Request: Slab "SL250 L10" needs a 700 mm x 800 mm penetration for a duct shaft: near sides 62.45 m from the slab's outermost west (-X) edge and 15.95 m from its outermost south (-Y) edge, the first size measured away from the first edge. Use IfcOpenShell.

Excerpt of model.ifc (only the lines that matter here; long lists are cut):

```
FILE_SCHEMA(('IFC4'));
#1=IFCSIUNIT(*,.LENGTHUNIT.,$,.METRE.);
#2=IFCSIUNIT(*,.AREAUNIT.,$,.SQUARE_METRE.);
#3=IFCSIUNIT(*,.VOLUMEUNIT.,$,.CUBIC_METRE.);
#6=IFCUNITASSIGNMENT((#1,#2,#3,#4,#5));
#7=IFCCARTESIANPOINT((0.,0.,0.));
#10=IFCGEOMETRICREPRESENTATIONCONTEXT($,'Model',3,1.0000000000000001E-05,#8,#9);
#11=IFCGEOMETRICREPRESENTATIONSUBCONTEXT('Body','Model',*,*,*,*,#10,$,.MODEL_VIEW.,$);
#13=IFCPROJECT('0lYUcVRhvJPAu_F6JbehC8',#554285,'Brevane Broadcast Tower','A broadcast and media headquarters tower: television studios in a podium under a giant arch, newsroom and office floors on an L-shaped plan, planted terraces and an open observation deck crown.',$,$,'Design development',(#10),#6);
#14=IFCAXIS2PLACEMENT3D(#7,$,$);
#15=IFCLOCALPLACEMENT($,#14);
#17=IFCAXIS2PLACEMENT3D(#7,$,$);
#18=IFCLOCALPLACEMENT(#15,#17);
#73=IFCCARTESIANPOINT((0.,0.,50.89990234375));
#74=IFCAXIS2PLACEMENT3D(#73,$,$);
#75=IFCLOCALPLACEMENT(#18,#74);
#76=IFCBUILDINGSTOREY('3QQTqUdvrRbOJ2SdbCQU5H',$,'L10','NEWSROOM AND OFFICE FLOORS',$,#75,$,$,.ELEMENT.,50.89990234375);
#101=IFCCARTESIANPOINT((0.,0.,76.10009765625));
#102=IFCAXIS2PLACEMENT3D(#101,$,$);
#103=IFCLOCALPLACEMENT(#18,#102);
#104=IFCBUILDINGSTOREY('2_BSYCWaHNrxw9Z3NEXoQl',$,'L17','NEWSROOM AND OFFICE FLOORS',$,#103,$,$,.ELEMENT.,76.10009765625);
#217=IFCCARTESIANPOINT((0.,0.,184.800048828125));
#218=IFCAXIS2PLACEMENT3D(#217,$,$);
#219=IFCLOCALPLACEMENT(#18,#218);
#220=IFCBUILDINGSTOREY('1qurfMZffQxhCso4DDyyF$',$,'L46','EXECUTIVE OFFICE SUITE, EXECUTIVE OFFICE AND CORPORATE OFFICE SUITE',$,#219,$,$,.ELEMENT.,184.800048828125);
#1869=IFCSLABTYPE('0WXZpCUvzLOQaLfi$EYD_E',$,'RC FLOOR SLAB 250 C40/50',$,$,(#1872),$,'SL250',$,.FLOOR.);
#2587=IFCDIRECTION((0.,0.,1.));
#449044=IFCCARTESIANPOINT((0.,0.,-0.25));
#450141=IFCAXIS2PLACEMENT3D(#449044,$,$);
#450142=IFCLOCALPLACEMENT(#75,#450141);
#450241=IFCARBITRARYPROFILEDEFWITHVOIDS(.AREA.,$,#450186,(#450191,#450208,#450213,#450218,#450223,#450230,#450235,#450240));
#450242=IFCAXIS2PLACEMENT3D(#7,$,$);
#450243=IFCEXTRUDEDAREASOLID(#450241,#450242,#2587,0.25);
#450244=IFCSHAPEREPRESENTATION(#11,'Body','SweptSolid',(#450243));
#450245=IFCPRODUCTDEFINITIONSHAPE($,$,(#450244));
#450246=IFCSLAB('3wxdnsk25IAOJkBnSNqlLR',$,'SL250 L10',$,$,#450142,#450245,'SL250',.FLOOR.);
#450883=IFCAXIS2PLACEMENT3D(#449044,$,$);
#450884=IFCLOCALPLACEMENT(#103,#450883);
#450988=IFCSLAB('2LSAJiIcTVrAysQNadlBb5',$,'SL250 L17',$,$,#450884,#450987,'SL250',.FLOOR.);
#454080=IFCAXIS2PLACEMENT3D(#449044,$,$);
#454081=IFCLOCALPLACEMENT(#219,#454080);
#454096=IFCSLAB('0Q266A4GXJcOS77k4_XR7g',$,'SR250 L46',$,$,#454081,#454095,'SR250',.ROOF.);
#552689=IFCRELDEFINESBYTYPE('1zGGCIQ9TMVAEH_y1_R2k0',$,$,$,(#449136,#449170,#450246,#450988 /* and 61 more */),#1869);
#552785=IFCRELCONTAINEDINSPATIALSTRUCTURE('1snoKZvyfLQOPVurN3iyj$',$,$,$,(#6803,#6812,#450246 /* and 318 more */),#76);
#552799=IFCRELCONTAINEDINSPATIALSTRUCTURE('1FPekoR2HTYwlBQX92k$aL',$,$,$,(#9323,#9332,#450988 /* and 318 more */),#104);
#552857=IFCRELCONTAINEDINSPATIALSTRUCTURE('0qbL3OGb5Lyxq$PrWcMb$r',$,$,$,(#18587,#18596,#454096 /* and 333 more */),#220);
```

```python
import numpy as np
import ifcopenshell
import ifcopenshell.api.feature
import ifcopenshell.api.geometry
import ifcopenshell.api.root
import ifcopenshell.geom
import ifcopenshell.util.placement
import ifcopenshell.util.representation
import ifcopenshell.util.shape
import ifcopenshell.util.unit

model = ifcopenshell.open("model.ifc")
unit_scale = ifcopenshell.util.unit.calculate_unit_scale(model)
settings = ifcopenshell.geom.settings()


def volume(element):
    """Net volume in cubic metres, openings subtracted."""
    shape = ifcopenshell.geom.create_shape(settings, element)
    return ifcopenshell.util.shape.get_volume(shape.geometry)


slab = model.by_id(450246)
before = volume(slab)

# Extent in the slab's own axes, in metres. The edges named are its -X and -Y sides.
slab_shape = ifcopenshell.geom.create_shape(settings, slab)
vertices = ifcopenshell.util.shape.get_vertices(slab_shape.geometry)
x_min, y_min, bottom = vertices.min(axis=0)
top = vertices[:, 2].max()

opening = ifcopenshell.api.root.create_entity(model, ifc_class="IfcOpeningElement", name="Duct shaft opening", predefined_type="OPENING")
context = ifcopenshell.util.representation.get_context(model, "Model", "Body", "MODEL_VIEW")
width, depth = 0.7, 0.8
outline = [(0.0, 0.0), (width, 0.0), (width, depth), (0.0, depth), (0.0, 0.0)]
# Overshoot both faces by 50 mm so the cut is clean.
shape = ifcopenshell.api.geometry.add_slab_representation(
    model, context=context, depth=top - bottom + 0.1, polyline=outline
)
ifcopenshell.api.geometry.assign_representation(model, product=opening, representation=shape)

matrix = ifcopenshell.util.placement.get_local_placement(slab.ObjectPlacement)
matrix[:, 3] = matrix @ np.append(np.array([x_min + 62.45, y_min + 15.95, bottom - 0.05]) / unit_scale, 1.0)
ifcopenshell.api.geometry.edit_object_placement(model, product=opening, matrix=matrix, is_si=False)
ifcopenshell.api.feature.add_feature(model, feature=opening, element=slab)

after = volume(slab)

print(f"slab volume {before:.3f} -> {after:.3f} m3")

model.write("model-out.ifc")
```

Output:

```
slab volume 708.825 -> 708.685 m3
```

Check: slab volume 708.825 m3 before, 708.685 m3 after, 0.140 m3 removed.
